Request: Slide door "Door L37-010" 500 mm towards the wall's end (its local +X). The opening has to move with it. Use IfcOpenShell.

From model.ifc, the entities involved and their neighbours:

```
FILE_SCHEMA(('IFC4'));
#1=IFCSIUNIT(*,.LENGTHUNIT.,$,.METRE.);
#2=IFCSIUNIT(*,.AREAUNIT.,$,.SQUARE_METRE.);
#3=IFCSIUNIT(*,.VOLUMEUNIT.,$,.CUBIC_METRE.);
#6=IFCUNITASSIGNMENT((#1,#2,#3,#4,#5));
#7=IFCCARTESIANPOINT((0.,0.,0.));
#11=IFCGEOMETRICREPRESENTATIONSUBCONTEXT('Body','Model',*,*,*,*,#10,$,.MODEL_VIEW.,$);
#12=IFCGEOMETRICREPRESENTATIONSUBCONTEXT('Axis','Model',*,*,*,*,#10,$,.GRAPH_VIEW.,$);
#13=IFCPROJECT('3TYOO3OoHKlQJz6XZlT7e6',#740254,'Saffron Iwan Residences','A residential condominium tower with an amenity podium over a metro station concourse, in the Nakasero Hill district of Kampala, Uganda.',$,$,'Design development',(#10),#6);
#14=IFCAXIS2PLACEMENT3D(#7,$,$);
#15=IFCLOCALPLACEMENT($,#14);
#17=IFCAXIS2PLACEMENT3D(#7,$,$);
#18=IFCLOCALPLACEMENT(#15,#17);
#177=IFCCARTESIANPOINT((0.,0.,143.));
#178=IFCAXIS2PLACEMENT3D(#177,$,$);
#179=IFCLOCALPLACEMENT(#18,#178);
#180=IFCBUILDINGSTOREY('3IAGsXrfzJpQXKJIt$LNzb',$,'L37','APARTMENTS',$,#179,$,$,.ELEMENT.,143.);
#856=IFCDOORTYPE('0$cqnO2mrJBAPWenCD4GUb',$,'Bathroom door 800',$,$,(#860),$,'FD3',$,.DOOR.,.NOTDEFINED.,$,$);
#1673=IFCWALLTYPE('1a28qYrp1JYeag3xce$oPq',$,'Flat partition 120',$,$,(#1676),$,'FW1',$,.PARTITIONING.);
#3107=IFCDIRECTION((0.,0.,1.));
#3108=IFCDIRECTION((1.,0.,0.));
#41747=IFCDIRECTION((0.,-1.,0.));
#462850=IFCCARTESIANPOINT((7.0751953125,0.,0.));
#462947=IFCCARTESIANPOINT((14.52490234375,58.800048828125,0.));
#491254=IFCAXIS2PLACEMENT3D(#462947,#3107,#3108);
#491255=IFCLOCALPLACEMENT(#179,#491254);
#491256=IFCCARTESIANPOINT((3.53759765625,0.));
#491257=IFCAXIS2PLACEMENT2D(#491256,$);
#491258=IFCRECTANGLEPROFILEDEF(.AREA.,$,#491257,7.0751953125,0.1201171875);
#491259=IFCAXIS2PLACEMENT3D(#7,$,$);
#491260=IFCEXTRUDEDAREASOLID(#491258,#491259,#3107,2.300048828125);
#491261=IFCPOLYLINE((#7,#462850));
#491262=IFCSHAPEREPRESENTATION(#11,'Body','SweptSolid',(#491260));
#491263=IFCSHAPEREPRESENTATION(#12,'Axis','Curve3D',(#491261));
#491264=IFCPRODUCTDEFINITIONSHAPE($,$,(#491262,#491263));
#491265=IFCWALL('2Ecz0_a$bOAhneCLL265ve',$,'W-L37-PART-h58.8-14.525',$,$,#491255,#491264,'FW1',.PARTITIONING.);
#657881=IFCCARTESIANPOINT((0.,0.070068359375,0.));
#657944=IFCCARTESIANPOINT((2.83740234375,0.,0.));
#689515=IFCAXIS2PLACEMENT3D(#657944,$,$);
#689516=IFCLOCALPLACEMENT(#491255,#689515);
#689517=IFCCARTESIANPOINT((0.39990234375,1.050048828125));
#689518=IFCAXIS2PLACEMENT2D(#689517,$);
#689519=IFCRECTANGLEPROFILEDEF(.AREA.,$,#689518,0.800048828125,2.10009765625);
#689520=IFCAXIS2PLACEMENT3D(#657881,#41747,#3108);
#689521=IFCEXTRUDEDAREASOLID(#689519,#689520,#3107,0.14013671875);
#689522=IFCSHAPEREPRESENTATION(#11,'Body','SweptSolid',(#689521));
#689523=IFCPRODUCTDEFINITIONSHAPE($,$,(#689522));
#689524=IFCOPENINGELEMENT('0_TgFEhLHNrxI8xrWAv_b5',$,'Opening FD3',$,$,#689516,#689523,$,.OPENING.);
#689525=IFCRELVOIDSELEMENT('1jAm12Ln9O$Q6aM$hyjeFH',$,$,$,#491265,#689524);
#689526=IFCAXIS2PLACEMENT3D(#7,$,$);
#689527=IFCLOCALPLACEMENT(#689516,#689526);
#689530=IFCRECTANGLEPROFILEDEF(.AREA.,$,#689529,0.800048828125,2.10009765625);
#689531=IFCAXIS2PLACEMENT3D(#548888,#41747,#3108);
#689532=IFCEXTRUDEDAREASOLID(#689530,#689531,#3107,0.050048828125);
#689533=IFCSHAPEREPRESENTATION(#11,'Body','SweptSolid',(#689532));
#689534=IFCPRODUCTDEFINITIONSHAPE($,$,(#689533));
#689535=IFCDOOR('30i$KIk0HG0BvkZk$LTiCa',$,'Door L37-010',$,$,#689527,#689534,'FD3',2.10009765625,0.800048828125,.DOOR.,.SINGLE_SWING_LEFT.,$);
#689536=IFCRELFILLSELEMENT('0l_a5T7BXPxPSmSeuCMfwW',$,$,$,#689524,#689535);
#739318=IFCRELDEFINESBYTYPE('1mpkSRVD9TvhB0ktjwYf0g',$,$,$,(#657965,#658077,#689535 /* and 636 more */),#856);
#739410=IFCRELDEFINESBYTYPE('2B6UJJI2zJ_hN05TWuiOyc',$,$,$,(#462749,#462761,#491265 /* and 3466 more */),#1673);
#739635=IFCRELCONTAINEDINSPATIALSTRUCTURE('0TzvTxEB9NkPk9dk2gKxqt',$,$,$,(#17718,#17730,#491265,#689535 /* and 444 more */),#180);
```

```python
import ifcopenshell
import ifcopenshell.api.geometry
import ifcopenshell.util.placement
import ifcopenshell.util.unit

model = ifcopenshell.open("model.ifc")
unit_scale = ifcopenshell.util.unit.calculate_unit_scale(model)

door = model.by_guid("30i$KIk0HG0BvkZk$LTiCa")
opening = door.FillsVoids[0].RelatingOpeningElement
wall = opening.VoidsElements[0].RelatingBuildingElement

wall_matrix = ifcopenshell.util.placement.get_local_placement(wall.ObjectPlacement)
shift = wall_matrix[:3, 0] * 0.5 / unit_scale
before = ifcopenshell.util.placement.get_local_placement(door.ObjectPlacement)[:3, 3].copy()

# The door is placed relative to its opening, so it follows when the opening moves.
matrix = ifcopenshell.util.placement.get_local_placement(opening.ObjectPlacement)
matrix[:3, 3] += shift
ifcopenshell.api.geometry.edit_object_placement(
    model, product=opening, matrix=matrix, is_si=False, should_transform_children=True
)

after = ifcopenshell.util.placement.get_local_placement(door.ObjectPlacement)[:3, 3]
print("door moved by", (after - before).round(3) + 0.0)

model.write("model_v2.ifc")
```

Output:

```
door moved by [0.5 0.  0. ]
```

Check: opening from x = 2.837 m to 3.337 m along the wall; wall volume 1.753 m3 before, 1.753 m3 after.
